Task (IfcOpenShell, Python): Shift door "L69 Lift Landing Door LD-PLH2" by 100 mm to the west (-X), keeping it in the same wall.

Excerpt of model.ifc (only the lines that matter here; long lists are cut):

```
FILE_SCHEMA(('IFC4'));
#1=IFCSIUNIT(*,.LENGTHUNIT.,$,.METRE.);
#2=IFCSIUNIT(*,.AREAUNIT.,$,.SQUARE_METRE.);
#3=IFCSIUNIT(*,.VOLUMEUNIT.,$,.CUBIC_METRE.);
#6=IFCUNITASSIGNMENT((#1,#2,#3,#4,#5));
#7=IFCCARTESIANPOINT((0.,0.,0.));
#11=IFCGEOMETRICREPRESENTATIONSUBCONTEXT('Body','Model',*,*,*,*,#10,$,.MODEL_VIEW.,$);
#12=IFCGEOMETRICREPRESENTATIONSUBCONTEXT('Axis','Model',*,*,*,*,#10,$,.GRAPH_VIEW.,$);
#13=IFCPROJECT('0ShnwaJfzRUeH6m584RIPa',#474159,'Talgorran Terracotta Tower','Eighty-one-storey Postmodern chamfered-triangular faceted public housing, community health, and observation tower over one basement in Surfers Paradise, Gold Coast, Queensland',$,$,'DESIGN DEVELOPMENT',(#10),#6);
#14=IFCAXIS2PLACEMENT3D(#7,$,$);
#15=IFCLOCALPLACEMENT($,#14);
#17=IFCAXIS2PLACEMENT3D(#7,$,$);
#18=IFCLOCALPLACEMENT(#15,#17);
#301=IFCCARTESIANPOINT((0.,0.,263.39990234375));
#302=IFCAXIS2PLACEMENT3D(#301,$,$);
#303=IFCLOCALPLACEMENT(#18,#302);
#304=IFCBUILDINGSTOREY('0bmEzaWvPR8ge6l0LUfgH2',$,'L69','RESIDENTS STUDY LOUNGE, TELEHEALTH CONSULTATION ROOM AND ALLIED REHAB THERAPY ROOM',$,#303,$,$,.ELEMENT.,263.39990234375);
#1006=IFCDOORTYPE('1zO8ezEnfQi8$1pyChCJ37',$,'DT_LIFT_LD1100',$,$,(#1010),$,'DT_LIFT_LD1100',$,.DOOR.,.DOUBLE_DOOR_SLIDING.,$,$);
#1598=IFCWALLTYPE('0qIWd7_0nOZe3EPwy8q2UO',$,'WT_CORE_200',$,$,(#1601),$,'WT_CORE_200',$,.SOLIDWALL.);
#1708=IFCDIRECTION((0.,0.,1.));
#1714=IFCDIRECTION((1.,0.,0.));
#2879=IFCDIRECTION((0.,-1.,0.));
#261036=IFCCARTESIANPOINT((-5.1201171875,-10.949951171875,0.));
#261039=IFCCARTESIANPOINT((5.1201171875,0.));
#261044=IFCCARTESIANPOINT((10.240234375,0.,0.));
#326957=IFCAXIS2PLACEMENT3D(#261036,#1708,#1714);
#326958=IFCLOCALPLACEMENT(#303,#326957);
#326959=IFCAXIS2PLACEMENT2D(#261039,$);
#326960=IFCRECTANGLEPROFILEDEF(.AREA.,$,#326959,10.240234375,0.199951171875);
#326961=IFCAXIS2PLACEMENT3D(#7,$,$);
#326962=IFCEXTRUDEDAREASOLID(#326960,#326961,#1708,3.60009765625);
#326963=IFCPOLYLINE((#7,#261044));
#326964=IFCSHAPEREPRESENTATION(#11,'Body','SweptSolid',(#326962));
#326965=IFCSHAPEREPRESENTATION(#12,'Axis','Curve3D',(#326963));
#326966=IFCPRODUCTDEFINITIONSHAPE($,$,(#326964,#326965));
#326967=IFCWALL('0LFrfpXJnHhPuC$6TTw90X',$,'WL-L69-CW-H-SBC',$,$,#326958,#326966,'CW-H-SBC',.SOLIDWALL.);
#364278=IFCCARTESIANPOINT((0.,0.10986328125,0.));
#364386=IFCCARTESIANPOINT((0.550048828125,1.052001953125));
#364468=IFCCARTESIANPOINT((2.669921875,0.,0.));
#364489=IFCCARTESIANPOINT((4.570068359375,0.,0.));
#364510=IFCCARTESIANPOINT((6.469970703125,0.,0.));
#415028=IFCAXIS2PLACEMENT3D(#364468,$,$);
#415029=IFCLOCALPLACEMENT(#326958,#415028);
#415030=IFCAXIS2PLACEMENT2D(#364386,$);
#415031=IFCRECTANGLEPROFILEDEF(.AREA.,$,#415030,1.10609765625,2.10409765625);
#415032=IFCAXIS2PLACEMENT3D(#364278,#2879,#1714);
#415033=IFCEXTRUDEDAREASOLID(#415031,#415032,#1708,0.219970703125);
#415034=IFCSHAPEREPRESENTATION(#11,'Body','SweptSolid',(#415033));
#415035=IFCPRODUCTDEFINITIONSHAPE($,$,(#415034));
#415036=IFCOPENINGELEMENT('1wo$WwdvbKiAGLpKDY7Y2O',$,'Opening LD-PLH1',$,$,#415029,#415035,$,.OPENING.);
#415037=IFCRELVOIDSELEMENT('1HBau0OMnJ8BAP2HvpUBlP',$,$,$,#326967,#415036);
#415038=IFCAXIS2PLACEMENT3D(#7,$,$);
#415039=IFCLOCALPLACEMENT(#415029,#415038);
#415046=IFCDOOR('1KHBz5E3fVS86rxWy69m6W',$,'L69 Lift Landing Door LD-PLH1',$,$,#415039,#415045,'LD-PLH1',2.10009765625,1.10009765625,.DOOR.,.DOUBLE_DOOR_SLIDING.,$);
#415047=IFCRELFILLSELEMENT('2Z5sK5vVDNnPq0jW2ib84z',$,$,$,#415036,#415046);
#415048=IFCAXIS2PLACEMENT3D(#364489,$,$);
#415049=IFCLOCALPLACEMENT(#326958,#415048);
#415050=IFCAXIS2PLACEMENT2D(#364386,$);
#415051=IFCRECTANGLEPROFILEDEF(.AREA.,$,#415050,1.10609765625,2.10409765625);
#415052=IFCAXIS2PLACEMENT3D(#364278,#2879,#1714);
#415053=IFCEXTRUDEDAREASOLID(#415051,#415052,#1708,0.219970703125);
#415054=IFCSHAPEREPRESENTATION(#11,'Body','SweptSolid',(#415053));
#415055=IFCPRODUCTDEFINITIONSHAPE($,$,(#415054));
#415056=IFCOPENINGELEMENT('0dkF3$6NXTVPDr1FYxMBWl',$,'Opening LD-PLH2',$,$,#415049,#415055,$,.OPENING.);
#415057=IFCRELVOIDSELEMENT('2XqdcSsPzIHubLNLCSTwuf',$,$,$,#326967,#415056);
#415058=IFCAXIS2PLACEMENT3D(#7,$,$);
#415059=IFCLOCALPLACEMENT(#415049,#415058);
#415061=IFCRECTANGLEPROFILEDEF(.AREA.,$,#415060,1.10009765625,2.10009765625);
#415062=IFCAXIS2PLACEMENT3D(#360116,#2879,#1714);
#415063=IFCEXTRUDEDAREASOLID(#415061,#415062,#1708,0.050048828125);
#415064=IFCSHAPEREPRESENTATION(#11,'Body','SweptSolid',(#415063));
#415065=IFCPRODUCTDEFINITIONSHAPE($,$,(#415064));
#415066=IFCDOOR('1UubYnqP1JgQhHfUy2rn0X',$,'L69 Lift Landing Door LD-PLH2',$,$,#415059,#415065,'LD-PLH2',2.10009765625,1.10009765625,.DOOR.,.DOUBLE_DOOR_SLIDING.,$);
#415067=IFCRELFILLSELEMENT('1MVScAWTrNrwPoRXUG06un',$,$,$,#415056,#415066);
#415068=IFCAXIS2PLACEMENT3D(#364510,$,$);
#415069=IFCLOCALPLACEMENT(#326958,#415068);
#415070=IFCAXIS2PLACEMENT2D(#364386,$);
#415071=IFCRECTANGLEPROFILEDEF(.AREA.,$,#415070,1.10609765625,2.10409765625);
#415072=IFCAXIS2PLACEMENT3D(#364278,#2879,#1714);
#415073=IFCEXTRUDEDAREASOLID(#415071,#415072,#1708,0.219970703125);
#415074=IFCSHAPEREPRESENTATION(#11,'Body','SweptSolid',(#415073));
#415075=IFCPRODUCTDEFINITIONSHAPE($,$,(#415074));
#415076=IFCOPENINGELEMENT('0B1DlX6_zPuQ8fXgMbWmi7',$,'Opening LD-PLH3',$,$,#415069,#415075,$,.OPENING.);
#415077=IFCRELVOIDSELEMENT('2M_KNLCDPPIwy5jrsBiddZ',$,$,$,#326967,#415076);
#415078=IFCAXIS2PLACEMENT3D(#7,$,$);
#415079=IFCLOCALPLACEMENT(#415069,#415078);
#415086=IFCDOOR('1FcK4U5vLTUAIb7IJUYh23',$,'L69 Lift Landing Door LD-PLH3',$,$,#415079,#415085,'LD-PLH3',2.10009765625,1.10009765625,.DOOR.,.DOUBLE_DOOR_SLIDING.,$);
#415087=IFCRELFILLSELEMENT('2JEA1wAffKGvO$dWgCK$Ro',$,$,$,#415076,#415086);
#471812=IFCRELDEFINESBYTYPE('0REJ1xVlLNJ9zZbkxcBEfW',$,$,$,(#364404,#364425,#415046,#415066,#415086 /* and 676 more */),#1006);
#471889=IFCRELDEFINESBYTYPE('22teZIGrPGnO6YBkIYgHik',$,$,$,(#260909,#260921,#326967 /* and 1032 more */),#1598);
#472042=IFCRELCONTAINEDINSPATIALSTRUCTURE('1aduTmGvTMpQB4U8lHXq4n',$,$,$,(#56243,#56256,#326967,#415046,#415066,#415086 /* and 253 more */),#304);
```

```python
import ifcopenshell
import ifcopenshell.api.geometry
import ifcopenshell.util.placement

model = ifcopenshell.open("model.ifc")

door = model.by_guid("1UubYnqP1JgQhHfUy2rn0X")
opening = door.FillsVoids[0].RelatingOpeningElement
wall = opening.VoidsElements[0].RelatingBuildingElement

wall_matrix = ifcopenshell.util.placement.get_local_placement(wall.ObjectPlacement)
shift = wall_matrix[:3, 0] * -0.1
before = ifcopenshell.util.placement.get_local_placement(door.ObjectPlacement)[:3, 3].copy()

# The door is placed relative to its opening, so it follows when the opening moves.
matrix = ifcopenshell.util.placement.get_local_placement(opening.ObjectPlacement)
matrix[:3, 3] += shift
ifcopenshell.api.geometry.edit_object_placement(
    model, product=opening, matrix=matrix, is_si=False, should_transform_children=True
)

after = ifcopenshell.util.placement.get_local_placement(door.ObjectPlacement)[:3, 3]
print("door moved by", (after - before).round(3) + 0.0)

model.write("model-out.ifc")
```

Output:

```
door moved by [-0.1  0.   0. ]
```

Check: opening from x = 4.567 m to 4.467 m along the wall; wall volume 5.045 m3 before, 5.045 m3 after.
